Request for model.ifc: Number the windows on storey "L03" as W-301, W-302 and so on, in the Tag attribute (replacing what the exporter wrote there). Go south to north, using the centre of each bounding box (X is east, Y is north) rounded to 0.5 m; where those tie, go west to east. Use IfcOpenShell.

First a look at what the model holds.

```python
import ifcopenshell
import ifcopenshell.util.element
import ifcopenshell.util.placement

model = ifcopenshell.open("model.ifc")
print(model.schema)
storey = next(s for s in model.by_type("IfcBuildingStorey") if s.Name == "L03")
windows = [e for e in ifcopenshell.util.element.get_decomposition(storey) if e.is_a("IfcWindow")]
for e in sorted(windows, key=lambda e: e.id()):
    origin = ifcopenshell.util.placement.get_local_placement(e.ObjectPlacement)[:3, 3]
    print(e.id(), e.Tag, e.Name, origin.round(2) + 0.0, sep=" | ")
```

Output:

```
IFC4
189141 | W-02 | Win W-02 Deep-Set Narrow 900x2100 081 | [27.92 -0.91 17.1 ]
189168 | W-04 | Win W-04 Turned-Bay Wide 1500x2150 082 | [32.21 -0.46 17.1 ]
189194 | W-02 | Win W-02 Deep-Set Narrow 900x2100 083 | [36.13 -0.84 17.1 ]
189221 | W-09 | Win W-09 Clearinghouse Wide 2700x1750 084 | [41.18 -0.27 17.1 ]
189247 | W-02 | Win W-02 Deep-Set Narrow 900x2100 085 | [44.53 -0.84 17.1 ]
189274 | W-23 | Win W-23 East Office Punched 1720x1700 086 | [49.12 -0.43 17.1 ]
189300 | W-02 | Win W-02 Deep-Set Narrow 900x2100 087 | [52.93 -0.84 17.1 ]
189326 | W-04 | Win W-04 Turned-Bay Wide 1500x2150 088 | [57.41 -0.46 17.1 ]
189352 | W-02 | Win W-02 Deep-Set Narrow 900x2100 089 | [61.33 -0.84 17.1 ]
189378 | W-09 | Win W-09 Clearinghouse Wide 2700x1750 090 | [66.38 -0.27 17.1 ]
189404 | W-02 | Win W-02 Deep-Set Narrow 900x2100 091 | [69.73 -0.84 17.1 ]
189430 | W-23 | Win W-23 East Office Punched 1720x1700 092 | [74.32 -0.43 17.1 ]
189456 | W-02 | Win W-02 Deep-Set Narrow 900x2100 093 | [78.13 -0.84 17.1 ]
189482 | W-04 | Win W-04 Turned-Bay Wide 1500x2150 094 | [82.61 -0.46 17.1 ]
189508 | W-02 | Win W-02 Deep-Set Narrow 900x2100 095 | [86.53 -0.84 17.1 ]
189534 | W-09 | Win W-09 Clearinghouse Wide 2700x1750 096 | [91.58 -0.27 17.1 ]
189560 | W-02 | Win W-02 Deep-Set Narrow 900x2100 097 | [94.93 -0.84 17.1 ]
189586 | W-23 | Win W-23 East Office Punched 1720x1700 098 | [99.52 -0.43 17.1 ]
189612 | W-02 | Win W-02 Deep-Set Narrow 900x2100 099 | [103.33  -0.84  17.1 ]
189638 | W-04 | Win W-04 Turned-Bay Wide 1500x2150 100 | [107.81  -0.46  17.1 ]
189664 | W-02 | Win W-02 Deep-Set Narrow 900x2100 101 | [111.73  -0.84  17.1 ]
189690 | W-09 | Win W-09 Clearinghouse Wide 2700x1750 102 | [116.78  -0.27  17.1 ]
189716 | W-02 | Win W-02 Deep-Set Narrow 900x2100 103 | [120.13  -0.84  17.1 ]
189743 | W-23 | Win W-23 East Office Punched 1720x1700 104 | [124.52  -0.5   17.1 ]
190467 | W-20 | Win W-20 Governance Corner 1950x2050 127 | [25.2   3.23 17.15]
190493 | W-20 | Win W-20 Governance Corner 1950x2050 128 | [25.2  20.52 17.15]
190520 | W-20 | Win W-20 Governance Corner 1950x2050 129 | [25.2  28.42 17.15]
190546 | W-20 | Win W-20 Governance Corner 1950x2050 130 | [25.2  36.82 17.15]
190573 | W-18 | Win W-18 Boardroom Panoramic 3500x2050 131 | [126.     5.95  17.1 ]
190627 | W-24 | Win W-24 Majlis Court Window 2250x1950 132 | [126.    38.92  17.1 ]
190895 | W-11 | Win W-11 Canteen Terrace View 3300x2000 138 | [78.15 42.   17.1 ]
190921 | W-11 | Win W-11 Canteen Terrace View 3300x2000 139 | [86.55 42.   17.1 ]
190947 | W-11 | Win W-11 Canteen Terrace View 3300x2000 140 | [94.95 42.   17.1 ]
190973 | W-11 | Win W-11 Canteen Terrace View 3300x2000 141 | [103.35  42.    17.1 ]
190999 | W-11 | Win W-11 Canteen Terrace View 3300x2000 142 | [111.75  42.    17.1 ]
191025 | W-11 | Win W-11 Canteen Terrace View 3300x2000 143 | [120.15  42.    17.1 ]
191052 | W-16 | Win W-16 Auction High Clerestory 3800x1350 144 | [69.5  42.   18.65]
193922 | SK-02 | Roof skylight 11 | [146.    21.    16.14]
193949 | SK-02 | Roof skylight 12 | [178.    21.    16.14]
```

```python
import ifcopenshell
import ifcopenshell.geom
import ifcopenshell.util.element
import ifcopenshell.util.shape

model = ifcopenshell.open("model.ifc")
settings = ifcopenshell.geom.settings()
settings.set("use-world-coords", True)


def centre(element):
    shape = ifcopenshell.geom.create_shape(settings, element)
    return ifcopenshell.util.shape.get_bbox_centroid(shape.geometry)


storey = next(s for s in model.by_type("IfcBuildingStorey") if s.Name == "L03")
windows = [e for e in ifcopenshell.util.element.get_decomposition(storey) if e.is_a("IfcWindow")]

# Insertion points can sit at a corner or the storey origin, so sort by the geometry (in metres).
centres = {e: centre(e) for e in windows}
windows.sort(key=lambda e: (round(centres[e][1] / 0.5), centres[e][0]))

for i, e in enumerate(windows, start=1):
    number = f"W-3{i:02d}"
    e.Tag = number
    print(e.id(), number)

model.write("model_rev.ifc")
```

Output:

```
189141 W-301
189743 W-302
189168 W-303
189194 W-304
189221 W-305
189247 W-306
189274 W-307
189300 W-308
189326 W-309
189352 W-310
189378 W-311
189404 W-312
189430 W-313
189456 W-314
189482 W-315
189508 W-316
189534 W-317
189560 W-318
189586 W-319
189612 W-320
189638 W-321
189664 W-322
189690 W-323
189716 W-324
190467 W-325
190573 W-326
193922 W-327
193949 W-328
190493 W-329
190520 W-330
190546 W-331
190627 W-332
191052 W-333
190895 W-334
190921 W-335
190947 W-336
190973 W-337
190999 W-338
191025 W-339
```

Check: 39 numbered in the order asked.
